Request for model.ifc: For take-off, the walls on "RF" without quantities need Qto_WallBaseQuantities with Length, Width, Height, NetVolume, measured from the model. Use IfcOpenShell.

First a look at what the model holds.

```python
import ifcopenshell
import ifcopenshell.util.element
import ifcopenshell.util.unit

model = ifcopenshell.open("model.ifc")
print(model.schema)
for unit_type in ("LENGTHUNIT", "AREAUNIT", "VOLUMEUNIT"):
    print(unit_type, ifcopenshell.util.unit.calculate_unit_scale(model, unit_type))
storey = next(s for s in model.by_type("IfcBuildingStorey") if s.Name == "RF")
walls = [e for e in ifcopenshell.util.element.get_decomposition(storey) if e.is_a("IfcWall")]
for e in sorted(walls, key=lambda e: e.id()):
    print(e.id(), e.is_a(), e.Name, list(ifcopenshell.util.element.get_psets(e, qtos_only=True)), sep=" | ")
```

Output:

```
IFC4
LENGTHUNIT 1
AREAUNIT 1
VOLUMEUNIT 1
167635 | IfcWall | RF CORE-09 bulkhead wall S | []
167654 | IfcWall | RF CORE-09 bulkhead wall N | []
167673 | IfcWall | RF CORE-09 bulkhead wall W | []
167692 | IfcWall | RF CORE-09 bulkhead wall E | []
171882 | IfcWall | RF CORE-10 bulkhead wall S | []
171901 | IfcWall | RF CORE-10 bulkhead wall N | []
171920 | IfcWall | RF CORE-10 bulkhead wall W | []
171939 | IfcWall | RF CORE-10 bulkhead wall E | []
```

```python
import ifcopenshell
import ifcopenshell.api.pset
import ifcopenshell.geom
import ifcopenshell.util.element
import ifcopenshell.util.shape
import ifcopenshell.util.unit

model = ifcopenshell.open("model.ifc")
unit_scale = ifcopenshell.util.unit.calculate_unit_scale(model)
volume_scale = ifcopenshell.util.unit.calculate_unit_scale(model, "VOLUMEUNIT")
settings = ifcopenshell.geom.settings()

storey = next(s for s in model.by_type("IfcBuildingStorey") if s.Name == "RF")
walls = [e for e in ifcopenshell.util.element.get_decomposition(storey) if e.is_a("IfcWall")]

for e in sorted(walls, key=lambda e: e.id()):
    if ifcopenshell.util.element.get_psets(e, qtos_only=True, should_inherit=False):
        continue
    # Geometry comes back in metres, in the element's own axes.
    shape = ifcopenshell.geom.create_shape(settings, e)
    values = {
        "Length": ifcopenshell.util.shape.get_x(shape.geometry) / unit_scale,
        "Width": ifcopenshell.util.shape.get_y(shape.geometry) / unit_scale,
        "Height": ifcopenshell.util.shape.get_z(shape.geometry) / unit_scale,
        "NetVolume": ifcopenshell.util.shape.get_volume(shape.geometry) / volume_scale,
    }
    qto = ifcopenshell.api.pset.add_qto(model, product=e, name="Qto_WallBaseQuantities")
    ifcopenshell.api.pset.edit_qto(model, qto=qto, properties=values)
    print(e.id(), {k: round(v, 3) for k, v in values.items()})

model.write("model_edited.ifc")
```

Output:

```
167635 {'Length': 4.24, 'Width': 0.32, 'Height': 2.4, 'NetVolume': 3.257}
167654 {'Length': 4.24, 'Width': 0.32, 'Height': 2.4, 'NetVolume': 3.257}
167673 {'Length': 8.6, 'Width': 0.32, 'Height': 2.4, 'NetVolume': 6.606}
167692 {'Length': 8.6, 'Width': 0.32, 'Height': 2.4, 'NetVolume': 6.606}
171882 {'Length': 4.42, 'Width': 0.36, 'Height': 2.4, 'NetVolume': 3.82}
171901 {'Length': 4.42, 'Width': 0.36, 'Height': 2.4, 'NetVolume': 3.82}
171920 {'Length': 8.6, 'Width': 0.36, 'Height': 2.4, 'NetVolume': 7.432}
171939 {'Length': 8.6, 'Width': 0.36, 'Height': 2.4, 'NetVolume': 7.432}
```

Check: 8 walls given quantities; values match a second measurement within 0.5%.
